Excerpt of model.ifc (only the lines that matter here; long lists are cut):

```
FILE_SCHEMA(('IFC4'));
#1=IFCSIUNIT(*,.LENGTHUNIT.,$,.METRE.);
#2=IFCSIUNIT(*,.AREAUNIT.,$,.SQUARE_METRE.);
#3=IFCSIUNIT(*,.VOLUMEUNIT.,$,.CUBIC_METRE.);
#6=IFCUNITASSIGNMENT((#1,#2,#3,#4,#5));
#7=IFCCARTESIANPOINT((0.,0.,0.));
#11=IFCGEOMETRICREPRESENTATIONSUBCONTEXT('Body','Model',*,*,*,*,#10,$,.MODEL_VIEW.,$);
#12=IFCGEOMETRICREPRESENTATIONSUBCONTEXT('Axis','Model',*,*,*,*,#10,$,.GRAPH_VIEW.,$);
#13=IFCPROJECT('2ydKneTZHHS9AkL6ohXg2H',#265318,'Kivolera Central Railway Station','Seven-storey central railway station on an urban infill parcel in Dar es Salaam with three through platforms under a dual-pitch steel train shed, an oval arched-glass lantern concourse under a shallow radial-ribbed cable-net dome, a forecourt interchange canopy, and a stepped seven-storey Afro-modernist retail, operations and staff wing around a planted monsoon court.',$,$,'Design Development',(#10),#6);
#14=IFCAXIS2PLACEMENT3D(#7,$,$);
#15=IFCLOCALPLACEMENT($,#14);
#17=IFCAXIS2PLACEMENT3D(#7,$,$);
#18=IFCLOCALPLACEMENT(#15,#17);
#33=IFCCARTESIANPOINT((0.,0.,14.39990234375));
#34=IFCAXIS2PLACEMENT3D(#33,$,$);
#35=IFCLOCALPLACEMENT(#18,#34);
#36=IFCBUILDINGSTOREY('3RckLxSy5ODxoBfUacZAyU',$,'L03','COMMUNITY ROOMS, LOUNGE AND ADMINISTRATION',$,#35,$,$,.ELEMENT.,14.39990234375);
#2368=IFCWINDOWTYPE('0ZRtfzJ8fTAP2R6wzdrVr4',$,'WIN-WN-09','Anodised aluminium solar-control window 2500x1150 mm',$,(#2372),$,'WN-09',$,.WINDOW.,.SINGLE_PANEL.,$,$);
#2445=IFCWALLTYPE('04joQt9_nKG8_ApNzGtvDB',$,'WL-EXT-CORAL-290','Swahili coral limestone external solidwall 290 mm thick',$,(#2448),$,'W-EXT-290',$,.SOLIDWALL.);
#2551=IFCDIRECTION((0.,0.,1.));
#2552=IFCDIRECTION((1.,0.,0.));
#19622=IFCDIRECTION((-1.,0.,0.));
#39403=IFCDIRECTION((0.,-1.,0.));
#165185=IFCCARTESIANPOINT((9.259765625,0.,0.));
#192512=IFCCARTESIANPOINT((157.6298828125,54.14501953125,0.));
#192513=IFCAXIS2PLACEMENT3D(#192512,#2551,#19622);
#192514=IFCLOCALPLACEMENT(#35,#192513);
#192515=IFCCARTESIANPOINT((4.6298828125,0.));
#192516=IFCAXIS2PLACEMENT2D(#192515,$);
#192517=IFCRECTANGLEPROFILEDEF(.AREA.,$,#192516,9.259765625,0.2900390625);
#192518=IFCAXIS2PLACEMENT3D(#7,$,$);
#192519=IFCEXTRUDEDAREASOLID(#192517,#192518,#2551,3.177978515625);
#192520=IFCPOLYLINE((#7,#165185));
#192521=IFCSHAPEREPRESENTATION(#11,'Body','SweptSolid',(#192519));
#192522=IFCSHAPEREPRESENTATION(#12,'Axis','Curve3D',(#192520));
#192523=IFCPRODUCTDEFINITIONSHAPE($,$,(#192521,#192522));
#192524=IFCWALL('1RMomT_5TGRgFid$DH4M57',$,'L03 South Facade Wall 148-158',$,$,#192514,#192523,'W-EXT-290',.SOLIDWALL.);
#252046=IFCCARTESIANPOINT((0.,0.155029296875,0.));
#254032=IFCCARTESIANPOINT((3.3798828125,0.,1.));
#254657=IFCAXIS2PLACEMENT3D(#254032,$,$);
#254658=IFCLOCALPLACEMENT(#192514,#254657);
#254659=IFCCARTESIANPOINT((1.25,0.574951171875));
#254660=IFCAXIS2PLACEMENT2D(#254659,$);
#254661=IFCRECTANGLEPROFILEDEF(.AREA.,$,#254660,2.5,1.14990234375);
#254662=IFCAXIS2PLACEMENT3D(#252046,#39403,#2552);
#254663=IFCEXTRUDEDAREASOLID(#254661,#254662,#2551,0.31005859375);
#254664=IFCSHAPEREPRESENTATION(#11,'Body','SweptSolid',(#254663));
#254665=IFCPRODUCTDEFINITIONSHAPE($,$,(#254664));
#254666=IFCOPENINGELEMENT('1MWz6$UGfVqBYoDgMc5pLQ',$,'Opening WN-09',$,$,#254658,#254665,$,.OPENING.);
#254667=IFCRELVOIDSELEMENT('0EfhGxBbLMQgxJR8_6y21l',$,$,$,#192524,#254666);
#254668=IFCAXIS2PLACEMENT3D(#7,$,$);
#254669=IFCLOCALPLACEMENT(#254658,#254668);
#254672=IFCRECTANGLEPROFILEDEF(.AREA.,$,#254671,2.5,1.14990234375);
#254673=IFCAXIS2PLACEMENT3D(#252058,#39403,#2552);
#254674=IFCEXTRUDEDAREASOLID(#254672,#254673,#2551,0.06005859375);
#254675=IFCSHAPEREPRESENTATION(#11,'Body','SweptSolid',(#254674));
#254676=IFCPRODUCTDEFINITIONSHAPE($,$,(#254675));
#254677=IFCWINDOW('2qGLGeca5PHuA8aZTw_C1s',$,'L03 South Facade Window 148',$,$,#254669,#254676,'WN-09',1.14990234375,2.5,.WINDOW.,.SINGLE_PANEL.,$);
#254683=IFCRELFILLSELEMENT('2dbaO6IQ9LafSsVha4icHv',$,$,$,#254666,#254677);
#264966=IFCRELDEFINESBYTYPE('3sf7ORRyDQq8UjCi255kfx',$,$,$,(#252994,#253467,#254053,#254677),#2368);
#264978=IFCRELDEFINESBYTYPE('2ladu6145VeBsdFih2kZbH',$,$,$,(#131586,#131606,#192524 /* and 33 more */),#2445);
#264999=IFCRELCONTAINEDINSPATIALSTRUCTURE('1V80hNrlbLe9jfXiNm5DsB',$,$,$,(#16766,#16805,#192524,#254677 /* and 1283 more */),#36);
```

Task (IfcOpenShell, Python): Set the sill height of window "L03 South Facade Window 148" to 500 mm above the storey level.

```python
import numpy as np
import ifcopenshell
import ifcopenshell.api.geometry
import ifcopenshell.geom
import ifcopenshell.util.element
import ifcopenshell.util.placement
import ifcopenshell.util.shape
import ifcopenshell.util.unit

model = ifcopenshell.open("model.ifc")
unit_scale = ifcopenshell.util.unit.calculate_unit_scale(model)

window = model.by_guid("2qGLGeca5PHuA8aZTw_C1s")
opening = window.FillsVoids[0].RelatingOpeningElement
storey = ifcopenshell.util.element.get_container(window, ifc_class="IfcBuildingStorey")
level = ifcopenshell.util.placement.get_local_placement(storey.ObjectPlacement)[2, 3]

# The opening's origin need not be at the sill, so measure its lowest point.
shape = ifcopenshell.geom.create_shape(ifcopenshell.geom.settings(), opening)
bottom = ifcopenshell.util.shape.get_shape_bottom_elevation(shape, shape.geometry) / unit_scale
dz = level + 0.5 / unit_scale - bottom

shift = np.array([0.0, 0.0, dz])
# The window is placed relative to its opening, so it follows when the opening moves.
matrix = ifcopenshell.util.placement.get_local_placement(opening.ObjectPlacement)
matrix[:3, 3] += shift
ifcopenshell.api.geometry.edit_object_placement(
    model, product=opening, matrix=matrix, is_si=False, should_transform_children=True
)

print(f"moved by {dz * unit_scale:+.3f} m")

model.write("model_edited.ifc")
```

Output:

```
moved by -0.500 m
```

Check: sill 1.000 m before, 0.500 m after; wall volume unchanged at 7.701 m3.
